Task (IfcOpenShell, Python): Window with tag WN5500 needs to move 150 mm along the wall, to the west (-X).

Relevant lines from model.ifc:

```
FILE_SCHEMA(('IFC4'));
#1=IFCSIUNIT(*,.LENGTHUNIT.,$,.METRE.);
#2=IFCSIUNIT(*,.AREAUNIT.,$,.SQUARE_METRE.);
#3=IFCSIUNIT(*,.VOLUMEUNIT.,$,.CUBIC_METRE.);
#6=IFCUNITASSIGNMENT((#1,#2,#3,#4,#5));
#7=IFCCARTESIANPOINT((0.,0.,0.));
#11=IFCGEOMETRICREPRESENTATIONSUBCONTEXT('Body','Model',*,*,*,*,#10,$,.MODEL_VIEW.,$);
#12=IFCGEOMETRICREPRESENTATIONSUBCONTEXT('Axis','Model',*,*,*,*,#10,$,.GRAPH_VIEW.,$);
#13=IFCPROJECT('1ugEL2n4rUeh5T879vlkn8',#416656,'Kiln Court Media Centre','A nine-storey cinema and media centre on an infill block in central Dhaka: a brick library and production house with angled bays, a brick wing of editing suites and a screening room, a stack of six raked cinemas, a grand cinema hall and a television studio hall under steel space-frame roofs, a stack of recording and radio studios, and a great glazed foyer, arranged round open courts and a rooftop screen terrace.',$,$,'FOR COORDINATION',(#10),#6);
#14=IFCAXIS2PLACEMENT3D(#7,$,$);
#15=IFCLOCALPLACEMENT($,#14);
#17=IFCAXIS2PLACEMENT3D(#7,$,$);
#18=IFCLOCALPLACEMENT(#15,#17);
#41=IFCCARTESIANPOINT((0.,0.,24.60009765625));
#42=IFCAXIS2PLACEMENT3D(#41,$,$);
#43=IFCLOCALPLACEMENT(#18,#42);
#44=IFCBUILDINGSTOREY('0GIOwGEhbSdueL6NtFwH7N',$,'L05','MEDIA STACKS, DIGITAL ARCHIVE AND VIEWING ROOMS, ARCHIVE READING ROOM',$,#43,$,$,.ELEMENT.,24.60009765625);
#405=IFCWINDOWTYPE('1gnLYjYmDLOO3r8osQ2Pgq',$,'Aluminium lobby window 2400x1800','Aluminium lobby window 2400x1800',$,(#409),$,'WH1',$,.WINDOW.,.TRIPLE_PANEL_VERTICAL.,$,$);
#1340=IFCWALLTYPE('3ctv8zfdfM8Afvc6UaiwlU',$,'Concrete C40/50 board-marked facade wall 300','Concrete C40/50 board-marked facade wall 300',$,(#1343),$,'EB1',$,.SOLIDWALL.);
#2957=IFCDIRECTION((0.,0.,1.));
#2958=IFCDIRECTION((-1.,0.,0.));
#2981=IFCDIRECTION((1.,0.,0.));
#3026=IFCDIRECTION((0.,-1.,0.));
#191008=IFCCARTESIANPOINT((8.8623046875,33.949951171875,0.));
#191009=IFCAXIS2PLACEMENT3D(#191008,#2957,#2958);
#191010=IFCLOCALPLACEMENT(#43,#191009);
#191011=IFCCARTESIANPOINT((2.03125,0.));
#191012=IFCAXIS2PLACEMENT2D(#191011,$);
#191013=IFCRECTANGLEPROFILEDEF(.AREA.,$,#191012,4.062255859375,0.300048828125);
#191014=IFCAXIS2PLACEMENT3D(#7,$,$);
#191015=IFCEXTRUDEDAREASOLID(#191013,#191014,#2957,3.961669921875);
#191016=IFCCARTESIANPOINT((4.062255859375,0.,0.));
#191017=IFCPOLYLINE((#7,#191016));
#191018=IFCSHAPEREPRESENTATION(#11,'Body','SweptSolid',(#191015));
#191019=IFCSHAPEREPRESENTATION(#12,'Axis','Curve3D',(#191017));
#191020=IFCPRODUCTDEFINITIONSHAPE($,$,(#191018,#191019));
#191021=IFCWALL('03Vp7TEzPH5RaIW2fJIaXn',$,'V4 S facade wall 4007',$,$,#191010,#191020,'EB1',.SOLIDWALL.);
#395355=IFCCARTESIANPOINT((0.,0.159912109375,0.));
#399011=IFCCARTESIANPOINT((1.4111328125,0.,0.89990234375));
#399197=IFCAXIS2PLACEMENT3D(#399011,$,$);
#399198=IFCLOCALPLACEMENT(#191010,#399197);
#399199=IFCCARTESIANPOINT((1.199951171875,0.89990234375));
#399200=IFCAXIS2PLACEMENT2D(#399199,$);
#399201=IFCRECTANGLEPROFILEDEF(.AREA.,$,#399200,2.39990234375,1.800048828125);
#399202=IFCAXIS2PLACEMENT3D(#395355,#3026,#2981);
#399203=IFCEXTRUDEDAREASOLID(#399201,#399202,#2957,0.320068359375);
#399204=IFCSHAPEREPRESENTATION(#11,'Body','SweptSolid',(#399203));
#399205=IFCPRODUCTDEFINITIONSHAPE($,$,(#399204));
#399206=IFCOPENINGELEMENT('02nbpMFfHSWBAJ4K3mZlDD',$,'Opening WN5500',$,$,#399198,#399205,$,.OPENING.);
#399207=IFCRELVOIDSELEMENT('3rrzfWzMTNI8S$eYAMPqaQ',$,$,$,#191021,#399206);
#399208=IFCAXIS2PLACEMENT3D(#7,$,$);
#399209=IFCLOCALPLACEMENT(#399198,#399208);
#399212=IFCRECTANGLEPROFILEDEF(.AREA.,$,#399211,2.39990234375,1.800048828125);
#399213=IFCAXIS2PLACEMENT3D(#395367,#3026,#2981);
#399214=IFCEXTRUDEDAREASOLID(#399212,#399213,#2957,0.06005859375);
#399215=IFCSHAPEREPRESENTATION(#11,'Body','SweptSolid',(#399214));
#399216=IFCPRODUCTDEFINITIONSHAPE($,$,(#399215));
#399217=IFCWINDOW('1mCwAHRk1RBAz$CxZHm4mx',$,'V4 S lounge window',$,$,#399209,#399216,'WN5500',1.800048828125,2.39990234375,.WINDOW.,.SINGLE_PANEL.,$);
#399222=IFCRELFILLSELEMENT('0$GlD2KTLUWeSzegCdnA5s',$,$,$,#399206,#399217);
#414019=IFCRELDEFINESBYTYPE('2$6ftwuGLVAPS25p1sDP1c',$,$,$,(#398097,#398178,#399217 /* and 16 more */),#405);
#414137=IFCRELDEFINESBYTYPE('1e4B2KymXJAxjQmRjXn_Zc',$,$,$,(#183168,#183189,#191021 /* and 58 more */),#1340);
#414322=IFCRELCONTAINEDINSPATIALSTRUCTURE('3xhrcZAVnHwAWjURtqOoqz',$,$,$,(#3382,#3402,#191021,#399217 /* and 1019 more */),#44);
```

```python
import ifcopenshell
import ifcopenshell.api.geometry
import ifcopenshell.util.placement
import ifcopenshell.util.unit

model = ifcopenshell.open("model.ifc")
unit_scale = ifcopenshell.util.unit.calculate_unit_scale(model)

window = model.by_guid("1mCwAHRk1RBAz$CxZHm4mx")
opening = window.FillsVoids[0].RelatingOpeningElement
wall = opening.VoidsElements[0].RelatingBuildingElement

wall_matrix = ifcopenshell.util.placement.get_local_placement(wall.ObjectPlacement)
shift = wall_matrix[:3, 0] * 0.15 / unit_scale
before = ifcopenshell.util.placement.get_local_placement(window.ObjectPlacement)[:3, 3].copy()

# The window is placed relative to its opening, so it follows when the opening moves.
matrix = ifcopenshell.util.placement.get_local_placement(opening.ObjectPlacement)
matrix[:3, 3] += shift
ifcopenshell.api.geometry.edit_object_placement(
    model, product=opening, matrix=matrix, is_si=False, should_transform_children=True
)

after = ifcopenshell.util.placement.get_local_placement(window.ObjectPlacement)[:3, 3]
print("window moved by", (after - before).round(3) + 0.0)

model.write("model-out.ifc")
```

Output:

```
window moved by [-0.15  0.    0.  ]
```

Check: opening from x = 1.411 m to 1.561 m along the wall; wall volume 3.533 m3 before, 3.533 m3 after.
